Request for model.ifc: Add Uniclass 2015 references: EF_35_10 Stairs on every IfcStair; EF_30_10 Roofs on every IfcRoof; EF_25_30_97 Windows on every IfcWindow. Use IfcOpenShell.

First a look at what the model holds.

```python
import ifcopenshell

model = ifcopenshell.open("model.ifc")
print(model.schema)
print("classifications:", [c.Name for c in model.by_type("IfcClassification")])
for ifc_class in ("IfcDoor", "IfcRoof", "IfcStair", "IfcWall", "IfcWindow"):
    print(ifc_class, len(model.by_type(ifc_class)))
```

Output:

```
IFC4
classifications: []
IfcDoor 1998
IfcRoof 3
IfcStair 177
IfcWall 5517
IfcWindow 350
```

```python
import ifcopenshell
import ifcopenshell.api.classification

model = ifcopenshell.open("model.ifc")

system = ifcopenshell.api.classification.add_classification(model, classification="Uniclass 2015")

codes = {
    "IfcStair": ("EF_35_10", "Stairs"),
    "IfcRoof": ("EF_30_10", "Roofs"),
    "IfcWindow": ("EF_25_30_97", "Windows"),
}
for ifc_class, (code, name) in codes.items():
    products = model.by_type(ifc_class)
    ifcopenshell.api.classification.add_reference(
        model, products=products, classification=system, identification=code, name=name
    )
    print(code, len(products))

model.write("model-out.ifc")
```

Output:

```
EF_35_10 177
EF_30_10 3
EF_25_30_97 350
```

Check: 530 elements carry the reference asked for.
